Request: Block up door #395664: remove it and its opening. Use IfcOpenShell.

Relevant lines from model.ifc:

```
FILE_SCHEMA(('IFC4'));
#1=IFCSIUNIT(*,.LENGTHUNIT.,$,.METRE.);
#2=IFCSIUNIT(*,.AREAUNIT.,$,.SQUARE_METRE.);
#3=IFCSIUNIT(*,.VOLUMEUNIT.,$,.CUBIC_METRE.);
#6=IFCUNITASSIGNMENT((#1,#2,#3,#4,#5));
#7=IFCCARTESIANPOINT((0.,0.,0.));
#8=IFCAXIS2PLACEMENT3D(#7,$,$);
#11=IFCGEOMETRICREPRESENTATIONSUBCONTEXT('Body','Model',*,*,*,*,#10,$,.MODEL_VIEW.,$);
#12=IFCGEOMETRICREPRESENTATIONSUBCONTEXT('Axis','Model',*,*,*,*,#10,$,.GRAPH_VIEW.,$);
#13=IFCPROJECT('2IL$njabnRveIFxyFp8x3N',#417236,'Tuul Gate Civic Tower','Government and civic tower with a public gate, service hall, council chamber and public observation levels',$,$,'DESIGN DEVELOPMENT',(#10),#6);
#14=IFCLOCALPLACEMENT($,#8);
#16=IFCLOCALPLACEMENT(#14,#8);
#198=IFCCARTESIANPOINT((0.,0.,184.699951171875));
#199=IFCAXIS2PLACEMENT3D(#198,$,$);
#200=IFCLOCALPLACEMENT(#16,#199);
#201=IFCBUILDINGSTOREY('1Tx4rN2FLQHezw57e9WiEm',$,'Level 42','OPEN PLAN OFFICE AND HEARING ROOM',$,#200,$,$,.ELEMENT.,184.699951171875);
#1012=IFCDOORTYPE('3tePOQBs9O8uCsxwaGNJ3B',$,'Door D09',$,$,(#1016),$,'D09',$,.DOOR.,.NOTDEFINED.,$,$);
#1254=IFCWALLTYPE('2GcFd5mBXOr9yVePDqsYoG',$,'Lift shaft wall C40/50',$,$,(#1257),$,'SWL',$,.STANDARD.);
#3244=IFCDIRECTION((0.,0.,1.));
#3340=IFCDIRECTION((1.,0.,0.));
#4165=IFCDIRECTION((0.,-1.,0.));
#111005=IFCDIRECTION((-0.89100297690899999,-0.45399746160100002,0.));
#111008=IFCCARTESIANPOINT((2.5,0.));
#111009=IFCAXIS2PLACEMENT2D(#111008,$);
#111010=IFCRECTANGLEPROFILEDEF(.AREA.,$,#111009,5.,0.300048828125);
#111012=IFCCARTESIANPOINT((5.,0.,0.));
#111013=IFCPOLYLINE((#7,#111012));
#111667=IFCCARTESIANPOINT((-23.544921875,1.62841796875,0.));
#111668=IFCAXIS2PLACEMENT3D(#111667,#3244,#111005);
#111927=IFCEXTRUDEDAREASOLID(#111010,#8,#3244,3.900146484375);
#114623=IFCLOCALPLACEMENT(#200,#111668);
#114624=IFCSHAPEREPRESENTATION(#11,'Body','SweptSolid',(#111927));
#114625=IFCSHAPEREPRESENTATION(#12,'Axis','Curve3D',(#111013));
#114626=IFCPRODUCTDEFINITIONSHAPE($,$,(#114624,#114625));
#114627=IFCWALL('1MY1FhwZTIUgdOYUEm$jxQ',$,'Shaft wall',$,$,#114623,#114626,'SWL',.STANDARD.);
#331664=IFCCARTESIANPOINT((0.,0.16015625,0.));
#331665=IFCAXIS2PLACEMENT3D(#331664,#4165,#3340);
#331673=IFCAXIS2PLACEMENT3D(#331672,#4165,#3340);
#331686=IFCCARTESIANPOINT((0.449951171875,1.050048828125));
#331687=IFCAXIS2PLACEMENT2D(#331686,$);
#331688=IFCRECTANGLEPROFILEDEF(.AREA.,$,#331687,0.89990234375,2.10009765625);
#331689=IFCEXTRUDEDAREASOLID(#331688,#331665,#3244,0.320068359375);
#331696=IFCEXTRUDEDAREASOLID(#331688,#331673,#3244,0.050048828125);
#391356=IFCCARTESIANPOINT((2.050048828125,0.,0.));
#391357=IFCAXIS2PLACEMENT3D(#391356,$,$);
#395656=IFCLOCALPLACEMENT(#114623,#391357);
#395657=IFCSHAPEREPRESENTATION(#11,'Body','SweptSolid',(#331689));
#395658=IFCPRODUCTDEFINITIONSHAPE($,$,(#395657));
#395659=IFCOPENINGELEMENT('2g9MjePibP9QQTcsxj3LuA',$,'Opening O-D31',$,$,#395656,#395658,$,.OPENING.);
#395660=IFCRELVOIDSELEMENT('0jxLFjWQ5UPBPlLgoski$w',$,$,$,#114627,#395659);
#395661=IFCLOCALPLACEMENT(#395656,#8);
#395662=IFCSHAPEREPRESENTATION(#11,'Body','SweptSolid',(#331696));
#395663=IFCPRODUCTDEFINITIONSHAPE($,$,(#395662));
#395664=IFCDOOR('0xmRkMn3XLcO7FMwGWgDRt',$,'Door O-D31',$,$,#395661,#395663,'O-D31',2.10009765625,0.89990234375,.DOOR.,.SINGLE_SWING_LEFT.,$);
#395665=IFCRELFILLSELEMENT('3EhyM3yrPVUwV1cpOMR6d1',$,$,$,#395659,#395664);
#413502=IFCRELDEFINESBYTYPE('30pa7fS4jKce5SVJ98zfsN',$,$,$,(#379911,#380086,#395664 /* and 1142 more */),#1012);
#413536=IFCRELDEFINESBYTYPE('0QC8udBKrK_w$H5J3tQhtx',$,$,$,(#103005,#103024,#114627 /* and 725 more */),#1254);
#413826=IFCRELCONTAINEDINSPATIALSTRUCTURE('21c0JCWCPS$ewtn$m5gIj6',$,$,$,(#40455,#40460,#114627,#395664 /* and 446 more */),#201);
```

```python
import ifcopenshell
import ifcopenshell.api.feature
import ifcopenshell.api.root
import ifcopenshell.geom
import ifcopenshell.util.shape

model = ifcopenshell.open("model.ifc")
settings = ifcopenshell.geom.settings()


def volume(element):
    """Net volume in cubic metres, openings subtracted."""
    shape = ifcopenshell.geom.create_shape(settings, element)
    return ifcopenshell.util.shape.get_volume(shape.geometry)


door = model.by_guid("0xmRkMn3XLcO7FMwGWgDRt")
opening = door.FillsVoids[0].RelatingOpeningElement
wall = opening.VoidsElements[0].RelatingBuildingElement
before = volume(wall)

ifcopenshell.api.root.remove_product(model, product=door)
ifcopenshell.api.feature.remove_feature(model, feature=opening)

after = volume(wall)

print(f"wall volume {before:.3f} -> {after:.3f} m3")

model.write("model-out.ifc")
```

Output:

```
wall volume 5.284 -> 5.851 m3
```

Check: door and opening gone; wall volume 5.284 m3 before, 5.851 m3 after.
